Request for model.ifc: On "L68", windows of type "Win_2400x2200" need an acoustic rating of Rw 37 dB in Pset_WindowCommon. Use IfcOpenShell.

First a look at what the model holds.

```python
import ifcopenshell
import ifcopenshell.util.element

model = ifcopenshell.open("model.ifc")
print(model.schema)
storey = next(s for s in model.by_type("IfcBuildingStorey") if s.Name == "L68")
windows = [e for e in ifcopenshell.util.element.get_decomposition(storey) if e.is_a("IfcWindow")]
seen = {}
for e in windows:
    element_type = ifcopenshell.util.element.get_type(e)
    key = (element_type.Name if element_type != e and element_type else None, ifcopenshell.util.element.get_pset(e, "Pset_WindowCommon", "AcousticRating"))
    seen[key] = seen.get(key, 0) + 1
for (name, value), count in sorted(seen.items(), key=str):
    print(count, "x", name, "|", value)
```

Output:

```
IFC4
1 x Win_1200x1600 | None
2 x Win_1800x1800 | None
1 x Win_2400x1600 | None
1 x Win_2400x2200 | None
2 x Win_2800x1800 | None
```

```python
import ifcopenshell
import ifcopenshell.api.pset
import ifcopenshell.util.element

model = ifcopenshell.open("model.ifc")

storey = next(s for s in model.by_type("IfcBuildingStorey") if s.Name == "L68")
windows = [e for e in ifcopenshell.util.element.get_decomposition(storey) if e.is_a("IfcWindow")]

count = 0
for e in windows:
    element_type = ifcopenshell.util.element.get_type(e)
    if element_type in (None, e) or element_type.Name != "Win_2400x2200":
        continue
    # add_pset returns the element's existing set when there is one.
    pset = ifcopenshell.api.pset.add_pset(model, product=e, name="Pset_WindowCommon")
    ifcopenshell.api.pset.edit_pset(model, pset=pset, properties={"AcousticRating": "Rw 37 dB"})
    count += 1

print(count, "windows updated")

model.write("model_updated.ifc")
```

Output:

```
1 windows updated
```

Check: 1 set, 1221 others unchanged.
